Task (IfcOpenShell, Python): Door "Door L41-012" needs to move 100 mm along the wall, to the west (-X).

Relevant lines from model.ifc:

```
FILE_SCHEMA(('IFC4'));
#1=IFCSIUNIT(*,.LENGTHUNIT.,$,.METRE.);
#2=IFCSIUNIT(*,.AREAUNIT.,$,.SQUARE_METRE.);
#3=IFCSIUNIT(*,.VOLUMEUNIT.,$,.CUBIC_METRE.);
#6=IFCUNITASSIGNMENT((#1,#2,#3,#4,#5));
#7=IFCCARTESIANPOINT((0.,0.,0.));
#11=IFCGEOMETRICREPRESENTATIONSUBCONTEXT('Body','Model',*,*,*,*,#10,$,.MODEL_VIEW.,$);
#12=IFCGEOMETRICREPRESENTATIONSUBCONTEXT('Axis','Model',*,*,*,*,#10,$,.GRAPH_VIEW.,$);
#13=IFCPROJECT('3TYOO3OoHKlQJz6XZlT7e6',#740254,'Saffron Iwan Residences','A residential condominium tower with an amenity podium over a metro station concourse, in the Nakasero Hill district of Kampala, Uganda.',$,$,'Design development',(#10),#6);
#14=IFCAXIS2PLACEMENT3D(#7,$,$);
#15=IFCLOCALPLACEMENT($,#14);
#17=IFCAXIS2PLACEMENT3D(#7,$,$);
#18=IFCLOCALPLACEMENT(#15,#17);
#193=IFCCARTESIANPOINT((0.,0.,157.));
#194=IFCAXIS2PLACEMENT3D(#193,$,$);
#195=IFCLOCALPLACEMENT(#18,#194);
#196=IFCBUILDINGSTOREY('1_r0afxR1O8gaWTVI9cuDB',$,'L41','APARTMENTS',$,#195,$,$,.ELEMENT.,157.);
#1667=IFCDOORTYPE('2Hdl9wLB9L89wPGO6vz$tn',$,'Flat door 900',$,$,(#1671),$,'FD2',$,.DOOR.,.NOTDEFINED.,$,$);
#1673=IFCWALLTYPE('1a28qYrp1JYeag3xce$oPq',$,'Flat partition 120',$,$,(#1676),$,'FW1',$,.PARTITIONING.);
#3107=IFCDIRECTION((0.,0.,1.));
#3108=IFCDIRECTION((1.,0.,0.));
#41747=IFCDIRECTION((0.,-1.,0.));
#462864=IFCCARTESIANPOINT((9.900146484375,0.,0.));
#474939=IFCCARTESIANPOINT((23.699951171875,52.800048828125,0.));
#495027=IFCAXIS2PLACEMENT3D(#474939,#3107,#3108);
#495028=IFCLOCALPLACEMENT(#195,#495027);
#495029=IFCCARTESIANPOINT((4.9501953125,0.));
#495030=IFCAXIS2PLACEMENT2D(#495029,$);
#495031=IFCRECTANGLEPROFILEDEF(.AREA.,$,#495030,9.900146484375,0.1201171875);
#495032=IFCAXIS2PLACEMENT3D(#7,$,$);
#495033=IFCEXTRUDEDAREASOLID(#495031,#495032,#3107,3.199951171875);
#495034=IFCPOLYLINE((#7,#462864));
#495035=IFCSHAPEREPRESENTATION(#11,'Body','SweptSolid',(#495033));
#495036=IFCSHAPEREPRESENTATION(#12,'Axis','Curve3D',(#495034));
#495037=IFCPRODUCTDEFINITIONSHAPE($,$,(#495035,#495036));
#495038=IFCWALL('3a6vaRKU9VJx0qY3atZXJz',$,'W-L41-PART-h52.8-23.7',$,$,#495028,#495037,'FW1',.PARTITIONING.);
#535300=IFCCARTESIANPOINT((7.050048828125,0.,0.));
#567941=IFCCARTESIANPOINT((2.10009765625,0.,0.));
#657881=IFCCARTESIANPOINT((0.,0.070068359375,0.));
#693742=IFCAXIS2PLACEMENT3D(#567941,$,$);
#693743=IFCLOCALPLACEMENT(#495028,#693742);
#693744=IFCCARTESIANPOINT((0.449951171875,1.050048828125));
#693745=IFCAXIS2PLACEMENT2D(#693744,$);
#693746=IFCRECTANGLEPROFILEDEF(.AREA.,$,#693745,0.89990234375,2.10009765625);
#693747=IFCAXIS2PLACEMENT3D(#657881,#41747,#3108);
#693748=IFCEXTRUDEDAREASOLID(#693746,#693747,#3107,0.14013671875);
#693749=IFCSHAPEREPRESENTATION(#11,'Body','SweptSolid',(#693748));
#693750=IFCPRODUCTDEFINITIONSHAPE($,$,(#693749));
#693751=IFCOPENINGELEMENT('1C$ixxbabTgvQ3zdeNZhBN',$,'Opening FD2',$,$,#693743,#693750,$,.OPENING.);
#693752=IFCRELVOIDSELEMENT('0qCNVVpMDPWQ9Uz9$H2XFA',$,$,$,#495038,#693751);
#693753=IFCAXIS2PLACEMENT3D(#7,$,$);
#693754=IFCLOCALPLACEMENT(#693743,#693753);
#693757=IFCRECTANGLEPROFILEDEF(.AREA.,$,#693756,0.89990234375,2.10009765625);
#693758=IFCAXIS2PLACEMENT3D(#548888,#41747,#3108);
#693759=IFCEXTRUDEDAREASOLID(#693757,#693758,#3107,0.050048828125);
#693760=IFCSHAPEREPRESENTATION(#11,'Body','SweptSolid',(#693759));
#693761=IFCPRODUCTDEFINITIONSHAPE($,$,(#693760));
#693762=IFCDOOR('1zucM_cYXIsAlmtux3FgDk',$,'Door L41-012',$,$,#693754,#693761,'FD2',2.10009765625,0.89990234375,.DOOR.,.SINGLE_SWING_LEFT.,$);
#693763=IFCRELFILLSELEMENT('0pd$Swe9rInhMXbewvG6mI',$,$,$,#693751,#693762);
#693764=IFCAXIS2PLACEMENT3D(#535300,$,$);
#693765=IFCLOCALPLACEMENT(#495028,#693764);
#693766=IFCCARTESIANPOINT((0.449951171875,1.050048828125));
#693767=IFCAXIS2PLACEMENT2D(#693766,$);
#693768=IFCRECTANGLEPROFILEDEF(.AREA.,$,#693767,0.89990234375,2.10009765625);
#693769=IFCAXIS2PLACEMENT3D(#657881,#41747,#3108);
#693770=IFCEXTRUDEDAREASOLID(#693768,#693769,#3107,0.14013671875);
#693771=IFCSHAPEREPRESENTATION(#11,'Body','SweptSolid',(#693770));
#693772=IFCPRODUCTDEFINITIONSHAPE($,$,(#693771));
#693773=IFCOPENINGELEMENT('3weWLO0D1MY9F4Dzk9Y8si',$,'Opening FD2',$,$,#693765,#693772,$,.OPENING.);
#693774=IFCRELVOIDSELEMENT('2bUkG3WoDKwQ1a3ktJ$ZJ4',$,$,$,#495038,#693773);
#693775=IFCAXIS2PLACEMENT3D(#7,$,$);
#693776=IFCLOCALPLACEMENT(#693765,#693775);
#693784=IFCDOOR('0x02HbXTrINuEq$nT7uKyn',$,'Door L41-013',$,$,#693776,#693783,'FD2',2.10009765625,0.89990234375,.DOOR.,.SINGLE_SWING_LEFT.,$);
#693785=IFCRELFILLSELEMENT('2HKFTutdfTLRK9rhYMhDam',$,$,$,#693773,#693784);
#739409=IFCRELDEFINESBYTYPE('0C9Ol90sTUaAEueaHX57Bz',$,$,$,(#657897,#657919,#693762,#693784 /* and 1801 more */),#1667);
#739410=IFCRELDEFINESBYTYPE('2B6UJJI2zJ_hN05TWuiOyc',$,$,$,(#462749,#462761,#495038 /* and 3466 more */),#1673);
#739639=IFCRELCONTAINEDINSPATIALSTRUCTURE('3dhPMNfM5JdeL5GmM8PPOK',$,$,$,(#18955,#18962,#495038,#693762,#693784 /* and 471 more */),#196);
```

```python
import ifcopenshell
import ifcopenshell.api.geometry
import ifcopenshell.util.placement
import ifcopenshell.util.unit

model = ifcopenshell.open("model.ifc")
unit_scale = ifcopenshell.util.unit.calculate_unit_scale(model)

door = model.by_guid("1zucM_cYXIsAlmtux3FgDk")
opening = door.FillsVoids[0].RelatingOpeningElement
wall = opening.VoidsElements[0].RelatingBuildingElement

wall_matrix = ifcopenshell.util.placement.get_local_placement(wall.ObjectPlacement)
shift = wall_matrix[:3, 0] * -0.1 / unit_scale
before = ifcopenshell.util.placement.get_local_placement(door.ObjectPlacement)[:3, 3].copy()

# The door is placed relative to its opening, so it follows when the opening moves.
matrix = ifcopenshell.util.placement.get_local_placement(opening.ObjectPlacement)
matrix[:3, 3] += shift
ifcopenshell.api.geometry.edit_object_placement(
    model, product=opening, matrix=matrix, is_si=False, should_transform_children=True
)

after = ifcopenshell.util.placement.get_local_placement(door.ObjectPlacement)[:3, 3]
print("door moved by", (after - before).round(3) + 0.0)

model.write("model_edited.ifc")
```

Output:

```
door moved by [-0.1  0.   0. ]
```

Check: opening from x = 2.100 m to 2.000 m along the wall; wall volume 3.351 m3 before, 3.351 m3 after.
